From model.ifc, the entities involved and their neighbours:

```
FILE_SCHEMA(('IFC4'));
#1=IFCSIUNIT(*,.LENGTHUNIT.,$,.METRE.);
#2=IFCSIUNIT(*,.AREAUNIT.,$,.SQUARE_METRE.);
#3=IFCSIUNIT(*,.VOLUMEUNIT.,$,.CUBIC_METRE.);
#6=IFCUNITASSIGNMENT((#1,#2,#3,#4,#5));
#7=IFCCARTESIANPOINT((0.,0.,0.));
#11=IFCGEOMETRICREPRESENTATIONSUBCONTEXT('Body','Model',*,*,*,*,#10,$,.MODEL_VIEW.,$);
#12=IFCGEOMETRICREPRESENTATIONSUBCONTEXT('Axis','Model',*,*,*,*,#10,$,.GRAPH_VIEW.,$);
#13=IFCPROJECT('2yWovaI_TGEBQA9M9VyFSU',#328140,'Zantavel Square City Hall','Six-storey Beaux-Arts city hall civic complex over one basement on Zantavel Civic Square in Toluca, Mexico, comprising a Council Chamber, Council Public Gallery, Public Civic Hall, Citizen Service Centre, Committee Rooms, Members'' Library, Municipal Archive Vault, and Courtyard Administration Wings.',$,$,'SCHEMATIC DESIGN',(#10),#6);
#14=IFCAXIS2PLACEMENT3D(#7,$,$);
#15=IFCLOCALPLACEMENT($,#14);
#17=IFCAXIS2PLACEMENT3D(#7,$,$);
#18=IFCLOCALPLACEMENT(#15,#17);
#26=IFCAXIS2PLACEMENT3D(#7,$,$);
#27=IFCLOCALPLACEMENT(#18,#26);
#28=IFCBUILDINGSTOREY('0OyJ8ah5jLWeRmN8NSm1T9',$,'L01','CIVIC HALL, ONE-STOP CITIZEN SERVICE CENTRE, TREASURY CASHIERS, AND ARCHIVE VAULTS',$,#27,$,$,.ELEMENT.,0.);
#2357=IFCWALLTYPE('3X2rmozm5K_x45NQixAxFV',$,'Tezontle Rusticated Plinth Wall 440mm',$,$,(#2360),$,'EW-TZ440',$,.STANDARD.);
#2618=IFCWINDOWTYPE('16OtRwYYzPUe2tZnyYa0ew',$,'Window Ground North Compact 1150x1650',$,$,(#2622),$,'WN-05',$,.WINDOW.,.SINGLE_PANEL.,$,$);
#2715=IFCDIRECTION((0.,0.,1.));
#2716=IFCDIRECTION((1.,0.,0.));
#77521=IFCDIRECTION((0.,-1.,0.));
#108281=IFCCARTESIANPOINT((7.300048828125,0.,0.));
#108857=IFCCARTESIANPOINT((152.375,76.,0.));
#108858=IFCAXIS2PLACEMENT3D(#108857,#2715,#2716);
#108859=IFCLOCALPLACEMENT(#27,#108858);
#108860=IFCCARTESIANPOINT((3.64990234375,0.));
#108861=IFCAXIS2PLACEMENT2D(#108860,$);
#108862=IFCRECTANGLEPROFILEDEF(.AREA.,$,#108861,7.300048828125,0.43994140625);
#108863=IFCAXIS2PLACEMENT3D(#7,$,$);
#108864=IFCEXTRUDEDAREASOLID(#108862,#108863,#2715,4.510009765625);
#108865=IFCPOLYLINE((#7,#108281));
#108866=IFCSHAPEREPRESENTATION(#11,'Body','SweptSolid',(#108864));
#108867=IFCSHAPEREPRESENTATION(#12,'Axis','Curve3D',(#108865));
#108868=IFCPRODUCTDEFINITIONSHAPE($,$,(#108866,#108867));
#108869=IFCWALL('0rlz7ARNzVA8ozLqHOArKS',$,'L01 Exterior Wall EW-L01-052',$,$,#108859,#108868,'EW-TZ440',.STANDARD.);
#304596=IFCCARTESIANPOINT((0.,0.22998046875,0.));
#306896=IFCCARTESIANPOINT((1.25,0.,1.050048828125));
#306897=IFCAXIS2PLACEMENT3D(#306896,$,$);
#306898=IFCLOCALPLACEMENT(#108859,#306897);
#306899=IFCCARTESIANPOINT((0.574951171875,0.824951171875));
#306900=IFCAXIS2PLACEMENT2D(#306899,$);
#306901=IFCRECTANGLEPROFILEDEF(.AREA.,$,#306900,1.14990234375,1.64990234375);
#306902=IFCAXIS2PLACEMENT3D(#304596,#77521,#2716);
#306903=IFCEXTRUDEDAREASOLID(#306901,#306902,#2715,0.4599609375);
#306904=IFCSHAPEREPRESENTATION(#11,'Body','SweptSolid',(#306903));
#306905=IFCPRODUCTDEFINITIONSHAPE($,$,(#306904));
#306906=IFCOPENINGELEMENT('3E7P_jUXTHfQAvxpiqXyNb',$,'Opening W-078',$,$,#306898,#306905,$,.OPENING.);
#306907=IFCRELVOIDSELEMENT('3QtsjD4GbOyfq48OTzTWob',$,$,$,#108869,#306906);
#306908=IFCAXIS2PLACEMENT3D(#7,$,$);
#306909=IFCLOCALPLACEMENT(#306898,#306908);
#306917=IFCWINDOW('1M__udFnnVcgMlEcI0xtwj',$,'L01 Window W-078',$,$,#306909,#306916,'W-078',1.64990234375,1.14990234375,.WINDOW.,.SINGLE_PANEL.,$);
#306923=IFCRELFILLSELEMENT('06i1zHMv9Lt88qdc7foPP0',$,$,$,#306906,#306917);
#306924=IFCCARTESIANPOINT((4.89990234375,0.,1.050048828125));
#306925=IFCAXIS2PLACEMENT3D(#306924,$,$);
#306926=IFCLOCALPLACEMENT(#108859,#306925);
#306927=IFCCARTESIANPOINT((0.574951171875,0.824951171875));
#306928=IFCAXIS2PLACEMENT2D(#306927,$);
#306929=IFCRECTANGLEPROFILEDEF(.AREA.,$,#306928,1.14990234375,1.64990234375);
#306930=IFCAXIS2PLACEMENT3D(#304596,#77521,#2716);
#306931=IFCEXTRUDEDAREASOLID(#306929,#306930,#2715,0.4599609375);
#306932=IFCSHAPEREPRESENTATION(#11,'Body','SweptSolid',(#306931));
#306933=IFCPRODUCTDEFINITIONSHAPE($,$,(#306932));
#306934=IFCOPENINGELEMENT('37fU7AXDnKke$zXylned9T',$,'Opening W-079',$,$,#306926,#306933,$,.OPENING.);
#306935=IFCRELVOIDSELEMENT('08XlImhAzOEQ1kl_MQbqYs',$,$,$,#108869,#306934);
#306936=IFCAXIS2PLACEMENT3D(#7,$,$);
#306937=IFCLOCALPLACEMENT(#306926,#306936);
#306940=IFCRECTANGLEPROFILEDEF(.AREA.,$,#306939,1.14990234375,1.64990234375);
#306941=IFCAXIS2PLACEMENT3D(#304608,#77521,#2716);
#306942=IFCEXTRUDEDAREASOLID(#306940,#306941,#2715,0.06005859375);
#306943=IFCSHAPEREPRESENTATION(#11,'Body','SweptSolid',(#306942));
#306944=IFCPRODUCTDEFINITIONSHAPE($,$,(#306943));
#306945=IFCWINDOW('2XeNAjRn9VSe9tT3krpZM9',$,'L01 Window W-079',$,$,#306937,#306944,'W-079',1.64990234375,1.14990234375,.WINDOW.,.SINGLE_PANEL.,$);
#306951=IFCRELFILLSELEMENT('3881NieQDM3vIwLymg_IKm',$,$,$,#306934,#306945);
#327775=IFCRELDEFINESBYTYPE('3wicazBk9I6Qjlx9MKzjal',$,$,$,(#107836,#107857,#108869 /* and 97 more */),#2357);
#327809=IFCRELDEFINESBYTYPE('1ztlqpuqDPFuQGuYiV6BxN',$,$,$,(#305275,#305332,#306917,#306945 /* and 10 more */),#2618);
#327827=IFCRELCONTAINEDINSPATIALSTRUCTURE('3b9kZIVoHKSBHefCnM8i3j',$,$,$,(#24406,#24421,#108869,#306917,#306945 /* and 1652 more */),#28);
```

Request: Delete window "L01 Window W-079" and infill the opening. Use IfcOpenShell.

```python
import ifcopenshell
import ifcopenshell.api.feature
import ifcopenshell.api.root
import ifcopenshell.geom
import ifcopenshell.util.shape

model = ifcopenshell.open("model.ifc")
settings = ifcopenshell.geom.settings()


def volume(element):
    """Net volume in cubic metres, openings subtracted."""
    shape = ifcopenshell.geom.create_shape(settings, element)
    return ifcopenshell.util.shape.get_volume(shape.geometry)


window = model.by_guid("2XeNAjRn9VSe9tT3krpZM9")
opening = window.FillsVoids[0].RelatingOpeningElement
wall = opening.VoidsElements[0].RelatingBuildingElement
before = volume(wall)

ifcopenshell.api.root.remove_product(model, product=window)
ifcopenshell.api.feature.remove_feature(model, feature=opening)

after = volume(wall)

print(f"wall volume {before:.3f} -> {after:.3f} m3")

model.write("model_v2.ifc")
```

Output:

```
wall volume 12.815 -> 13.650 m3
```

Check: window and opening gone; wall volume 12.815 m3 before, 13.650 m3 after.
